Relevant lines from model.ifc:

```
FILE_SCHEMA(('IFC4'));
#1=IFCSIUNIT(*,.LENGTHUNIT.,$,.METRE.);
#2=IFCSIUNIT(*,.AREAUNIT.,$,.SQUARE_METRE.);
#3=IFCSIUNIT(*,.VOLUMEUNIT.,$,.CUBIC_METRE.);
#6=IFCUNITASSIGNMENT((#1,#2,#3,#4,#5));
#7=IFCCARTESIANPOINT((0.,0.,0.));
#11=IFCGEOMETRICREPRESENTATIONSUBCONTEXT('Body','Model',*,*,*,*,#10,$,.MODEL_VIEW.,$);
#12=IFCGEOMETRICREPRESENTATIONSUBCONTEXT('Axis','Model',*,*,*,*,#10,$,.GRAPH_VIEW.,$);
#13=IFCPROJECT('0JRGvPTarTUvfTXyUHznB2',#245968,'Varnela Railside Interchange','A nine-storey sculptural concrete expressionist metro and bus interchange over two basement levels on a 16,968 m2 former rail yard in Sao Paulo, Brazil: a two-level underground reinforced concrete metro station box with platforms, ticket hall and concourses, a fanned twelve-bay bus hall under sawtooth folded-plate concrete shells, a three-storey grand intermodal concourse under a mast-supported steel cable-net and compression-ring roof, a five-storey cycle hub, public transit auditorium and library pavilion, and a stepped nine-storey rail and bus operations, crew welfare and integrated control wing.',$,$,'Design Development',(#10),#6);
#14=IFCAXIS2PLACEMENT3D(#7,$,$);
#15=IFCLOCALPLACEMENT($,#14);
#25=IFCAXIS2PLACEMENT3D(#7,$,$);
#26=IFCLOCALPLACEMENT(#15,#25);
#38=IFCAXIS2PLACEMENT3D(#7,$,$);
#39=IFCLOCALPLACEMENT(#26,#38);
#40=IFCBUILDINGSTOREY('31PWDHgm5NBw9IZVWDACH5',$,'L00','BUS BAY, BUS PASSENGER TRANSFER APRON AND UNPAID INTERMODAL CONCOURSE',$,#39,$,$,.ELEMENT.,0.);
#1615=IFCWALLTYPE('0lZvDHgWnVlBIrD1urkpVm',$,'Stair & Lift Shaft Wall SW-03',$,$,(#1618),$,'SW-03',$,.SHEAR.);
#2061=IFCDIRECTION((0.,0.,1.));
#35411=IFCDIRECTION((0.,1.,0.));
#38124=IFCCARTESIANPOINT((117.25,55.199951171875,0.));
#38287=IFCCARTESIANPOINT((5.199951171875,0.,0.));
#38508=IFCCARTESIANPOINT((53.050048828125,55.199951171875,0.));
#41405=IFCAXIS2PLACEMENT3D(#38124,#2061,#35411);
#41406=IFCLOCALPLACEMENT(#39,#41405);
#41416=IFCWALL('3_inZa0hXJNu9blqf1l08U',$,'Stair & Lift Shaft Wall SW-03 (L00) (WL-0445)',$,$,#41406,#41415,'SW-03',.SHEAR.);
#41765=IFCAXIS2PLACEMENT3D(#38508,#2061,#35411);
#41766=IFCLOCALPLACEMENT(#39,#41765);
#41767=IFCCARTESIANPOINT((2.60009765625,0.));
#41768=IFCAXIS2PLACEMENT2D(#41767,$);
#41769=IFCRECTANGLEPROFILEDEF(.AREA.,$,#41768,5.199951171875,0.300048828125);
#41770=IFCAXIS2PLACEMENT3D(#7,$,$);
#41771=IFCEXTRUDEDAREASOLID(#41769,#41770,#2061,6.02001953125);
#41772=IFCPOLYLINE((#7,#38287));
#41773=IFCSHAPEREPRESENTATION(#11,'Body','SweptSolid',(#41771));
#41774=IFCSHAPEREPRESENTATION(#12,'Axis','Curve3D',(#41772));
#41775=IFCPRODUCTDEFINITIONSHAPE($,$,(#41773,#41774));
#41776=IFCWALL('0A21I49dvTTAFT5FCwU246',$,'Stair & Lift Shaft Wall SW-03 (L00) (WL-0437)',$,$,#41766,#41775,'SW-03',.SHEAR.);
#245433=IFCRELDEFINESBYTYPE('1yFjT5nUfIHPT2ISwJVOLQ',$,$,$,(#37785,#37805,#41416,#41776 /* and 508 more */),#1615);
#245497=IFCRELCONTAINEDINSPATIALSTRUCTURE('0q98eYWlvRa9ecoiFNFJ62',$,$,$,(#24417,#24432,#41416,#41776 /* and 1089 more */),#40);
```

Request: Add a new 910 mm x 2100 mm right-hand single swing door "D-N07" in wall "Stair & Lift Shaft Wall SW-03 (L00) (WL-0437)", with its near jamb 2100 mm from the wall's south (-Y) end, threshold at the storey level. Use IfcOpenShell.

```python
import numpy as np
import ifcopenshell
import ifcopenshell.api.feature
import ifcopenshell.api.geometry
import ifcopenshell.api.root
import ifcopenshell.api.spatial
import ifcopenshell.geom
import ifcopenshell.util.element
import ifcopenshell.util.placement
import ifcopenshell.util.representation
import ifcopenshell.util.shape
import ifcopenshell.util.unit

model = ifcopenshell.open("model.ifc")
unit_scale = ifcopenshell.util.unit.calculate_unit_scale(model)
settings = ifcopenshell.geom.settings()


def volume(element):
    """Net volume in cubic metres, openings subtracted."""
    shape = ifcopenshell.geom.create_shape(settings, element)
    return ifcopenshell.util.shape.get_volume(shape.geometry)


wall = model.by_id(41776)
storey = ifcopenshell.util.element.get_container(wall, ifc_class="IfcBuildingStorey")
context = ifcopenshell.util.representation.get_context(model, "Model", "Body", "MODEL_VIEW")
before = volume(wall)

width, height, from_end, sill = 0.91, 2.1, 2.1, 0.0  # metres

# The wall runs along its own X axis, and the end named is its -X end.
wall_shape = ifcopenshell.geom.create_shape(settings, wall)
x, y, z = ifcopenshell.util.shape.get_vertices(wall_shape.geometry).T
start = x.min() + from_end
face, thickness = float(y.min()), float(y.max() - y.min())
wall_matrix = ifcopenshell.util.placement.get_local_placement(wall.ObjectPlacement)
level = ifcopenshell.util.placement.get_local_placement(storey.ObjectPlacement)[2, 3]


def in_wall(x, y):
    """Placement at x, y metres in the wall's axes, at sill height."""
    matrix = wall_matrix.copy()
    matrix[:, 3] = wall_matrix @ np.array([x / unit_scale, y / unit_scale, 0.0, 1.0])
    matrix[2, 3] = level + sill / unit_scale
    return matrix


# Opening: a box that overshoots both wall faces by 50 mm.
opening = ifcopenshell.api.root.create_entity(model, ifc_class="IfcOpeningElement", predefined_type="OPENING")
box = ifcopenshell.api.geometry.add_wall_representation(
    model, context=context, length=width, height=height, thickness=thickness + 0.1
)
ifcopenshell.api.geometry.assign_representation(model, product=opening, representation=box)
ifcopenshell.api.geometry.edit_object_placement(model, product=opening, matrix=in_wall(start, face - 0.05), is_si=False)
ifcopenshell.api.feature.add_feature(model, feature=opening, element=wall)

door = ifcopenshell.api.root.create_entity(model, ifc_class="IfcDoor", name="D-N07", predefined_type="DOOR")
door.OverallWidth, door.OverallHeight = width / unit_scale, height / unit_scale
door.OperationType = "SINGLE_SWING_RIGHT"
body = ifcopenshell.api.geometry.add_door_representation(
    model,
    context=context,
    overall_width=door.OverallWidth,
    overall_height=door.OverallHeight,
    operation_type="SINGLE_SWING_RIGHT",
    lining_properties={"LiningDepth": thickness / unit_scale, "ThresholdDepth": thickness / unit_scale},
)
ifcopenshell.api.geometry.assign_representation(model, product=door, representation=body)
ifcopenshell.api.spatial.assign_container(model, products=[door], relating_structure=storey)
ifcopenshell.api.feature.add_filling(model, opening=opening, element=door)

# The lining spans the wall, so the door starts at the wall face.
ifcopenshell.api.geometry.edit_object_placement(model, product=door, matrix=in_wall(start, face), is_si=False)

after = volume(wall)

print(f"wall volume {before:.3f} -> {after:.3f} m3")

model.write("model-out.ifc")
```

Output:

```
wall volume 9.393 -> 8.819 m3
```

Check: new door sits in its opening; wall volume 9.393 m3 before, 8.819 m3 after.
